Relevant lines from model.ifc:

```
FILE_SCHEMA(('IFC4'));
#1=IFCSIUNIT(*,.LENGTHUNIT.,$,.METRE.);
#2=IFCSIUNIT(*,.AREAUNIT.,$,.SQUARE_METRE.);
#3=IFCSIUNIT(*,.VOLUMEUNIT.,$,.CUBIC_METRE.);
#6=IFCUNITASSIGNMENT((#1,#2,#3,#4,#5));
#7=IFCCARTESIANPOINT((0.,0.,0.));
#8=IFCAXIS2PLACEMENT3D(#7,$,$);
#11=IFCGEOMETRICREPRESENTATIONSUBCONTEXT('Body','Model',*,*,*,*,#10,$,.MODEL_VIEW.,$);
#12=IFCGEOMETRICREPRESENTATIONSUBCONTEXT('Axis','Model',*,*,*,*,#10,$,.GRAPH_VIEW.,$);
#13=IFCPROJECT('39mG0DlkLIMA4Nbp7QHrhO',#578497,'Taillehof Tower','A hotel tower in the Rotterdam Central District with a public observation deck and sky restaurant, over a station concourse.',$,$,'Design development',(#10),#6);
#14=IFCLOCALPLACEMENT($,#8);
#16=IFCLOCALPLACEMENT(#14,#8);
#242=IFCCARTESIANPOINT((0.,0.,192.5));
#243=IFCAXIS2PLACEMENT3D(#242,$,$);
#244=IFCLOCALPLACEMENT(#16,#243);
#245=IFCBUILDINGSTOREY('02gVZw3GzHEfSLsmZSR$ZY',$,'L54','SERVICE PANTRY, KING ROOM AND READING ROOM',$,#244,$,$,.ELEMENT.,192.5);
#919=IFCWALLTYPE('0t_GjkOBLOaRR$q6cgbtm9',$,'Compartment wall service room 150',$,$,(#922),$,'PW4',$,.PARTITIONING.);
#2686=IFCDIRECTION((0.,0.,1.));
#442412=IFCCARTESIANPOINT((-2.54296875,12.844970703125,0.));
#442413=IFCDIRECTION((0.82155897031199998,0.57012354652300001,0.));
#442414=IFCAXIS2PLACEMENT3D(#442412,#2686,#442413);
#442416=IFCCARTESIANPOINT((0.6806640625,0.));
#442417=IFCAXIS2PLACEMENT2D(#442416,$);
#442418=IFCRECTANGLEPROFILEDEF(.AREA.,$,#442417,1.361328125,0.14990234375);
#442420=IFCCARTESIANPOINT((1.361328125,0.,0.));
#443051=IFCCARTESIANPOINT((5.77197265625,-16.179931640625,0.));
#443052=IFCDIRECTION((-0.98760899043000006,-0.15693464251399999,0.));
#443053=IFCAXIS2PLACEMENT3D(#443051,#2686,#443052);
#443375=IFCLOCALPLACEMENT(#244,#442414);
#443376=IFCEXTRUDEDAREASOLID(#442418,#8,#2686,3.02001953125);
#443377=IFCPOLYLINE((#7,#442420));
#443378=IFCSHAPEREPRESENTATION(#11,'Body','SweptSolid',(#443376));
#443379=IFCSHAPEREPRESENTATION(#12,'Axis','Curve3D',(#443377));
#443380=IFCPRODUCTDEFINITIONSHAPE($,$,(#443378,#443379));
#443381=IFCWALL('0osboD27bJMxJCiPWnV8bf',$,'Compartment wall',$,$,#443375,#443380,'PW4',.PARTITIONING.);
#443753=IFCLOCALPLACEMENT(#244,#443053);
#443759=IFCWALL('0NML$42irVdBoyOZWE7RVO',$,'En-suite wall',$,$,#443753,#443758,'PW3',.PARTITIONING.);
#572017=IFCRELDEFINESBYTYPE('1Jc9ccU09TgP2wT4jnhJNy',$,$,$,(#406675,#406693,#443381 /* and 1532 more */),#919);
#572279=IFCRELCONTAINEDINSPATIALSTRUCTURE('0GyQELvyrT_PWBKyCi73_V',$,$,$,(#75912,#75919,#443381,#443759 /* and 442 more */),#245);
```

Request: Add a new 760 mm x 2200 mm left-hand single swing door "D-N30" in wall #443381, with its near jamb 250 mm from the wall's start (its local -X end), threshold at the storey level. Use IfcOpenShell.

```python
import numpy as np
import ifcopenshell
import ifcopenshell.api.feature
import ifcopenshell.api.geometry
import ifcopenshell.api.root
import ifcopenshell.api.spatial
import ifcopenshell.geom
import ifcopenshell.util.element
import ifcopenshell.util.placement
import ifcopenshell.util.representation
import ifcopenshell.util.shape
import ifcopenshell.util.unit

model = ifcopenshell.open("model.ifc")
unit_scale = ifcopenshell.util.unit.calculate_unit_scale(model)
settings = ifcopenshell.geom.settings()


def volume(element):
    """Net volume in cubic metres, openings subtracted."""
    shape = ifcopenshell.geom.create_shape(settings, element)
    return ifcopenshell.util.shape.get_volume(shape.geometry)


wall = model.by_guid("0osboD27bJMxJCiPWnV8bf")
storey = ifcopenshell.util.element.get_container(wall, ifc_class="IfcBuildingStorey")
context = ifcopenshell.util.representation.get_context(model, "Model", "Body", "MODEL_VIEW")
before = volume(wall)

width, height, from_end, sill = 0.76, 2.2, 0.25, 0.0  # metres

# The wall runs along its own X axis, and the end named is its -X end.
wall_shape = ifcopenshell.geom.create_shape(settings, wall)
x, y, z = ifcopenshell.util.shape.get_vertices(wall_shape.geometry).T
start = x.min() + from_end
face, thickness = float(y.min()), float(y.max() - y.min())
wall_matrix = ifcopenshell.util.placement.get_local_placement(wall.ObjectPlacement)
level = ifcopenshell.util.placement.get_local_placement(storey.ObjectPlacement)[2, 3]


def in_wall(x, y):
    """Placement at x, y metres in the wall's axes, at sill height."""
    matrix = wall_matrix.copy()
    matrix[:, 3] = wall_matrix @ np.array([x / unit_scale, y / unit_scale, 0.0, 1.0])
    matrix[2, 3] = level + sill / unit_scale
    return matrix


# Opening: a box that overshoots both wall faces by 50 mm.
opening = ifcopenshell.api.root.create_entity(model, ifc_class="IfcOpeningElement", predefined_type="OPENING")
box = ifcopenshell.api.geometry.add_wall_representation(
    model, context=context, length=width, height=height, thickness=thickness + 0.1
)
ifcopenshell.api.geometry.assign_representation(model, product=opening, representation=box)
ifcopenshell.api.geometry.edit_object_placement(model, product=opening, matrix=in_wall(start, face - 0.05), is_si=False)
ifcopenshell.api.feature.add_feature(model, feature=opening, element=wall)

door = ifcopenshell.api.root.create_entity(model, ifc_class="IfcDoor", name="D-N30", predefined_type="DOOR")
door.OverallWidth, door.OverallHeight = width / unit_scale, height / unit_scale
door.OperationType = "SINGLE_SWING_LEFT"
body = ifcopenshell.api.geometry.add_door_representation(
    model,
    context=context,
    overall_width=door.OverallWidth,
    overall_height=door.OverallHeight,
    operation_type="SINGLE_SWING_LEFT",
    lining_properties={"LiningDepth": thickness / unit_scale, "ThresholdDepth": thickness / unit_scale},
)
ifcopenshell.api.geometry.assign_representation(model, product=door, representation=body)
ifcopenshell.api.spatial.assign_container(model, products=[door], relating_structure=storey)
ifcopenshell.api.feature.add_filling(model, opening=opening, element=door)

# The lining spans the wall, so the door starts at the wall face.
ifcopenshell.api.geometry.edit_object_placement(model, product=door, matrix=in_wall(start, face), is_si=False)

after = volume(wall)

print(f"wall volume {before:.3f} -> {after:.3f} m3")

model.write("model_edited.ifc")
```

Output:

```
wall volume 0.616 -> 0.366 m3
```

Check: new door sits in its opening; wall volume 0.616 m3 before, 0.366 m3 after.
